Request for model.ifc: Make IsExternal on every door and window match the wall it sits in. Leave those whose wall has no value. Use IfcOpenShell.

First a look at what the model holds.

```python
import ifcopenshell
import ifcopenshell.util.element

model = ifcopenshell.open("model.ifc")
print(model.schema)
seen = {}
for e in model.by_type("IfcDoor") + model.by_type("IfcWindow"):
    if not e.FillsVoids:
        continue
    host = e.FillsVoids[0].RelatingOpeningElement.VoidsElements[0].RelatingBuildingElement
    own = ifcopenshell.util.element.get_pset(e, f"Pset_{e.is_a()[3:].removesuffix('StandardCase')}Common", "IsExternal")
    wall = ifcopenshell.util.element.get_pset(host, "Pset_WallCommon", "IsExternal")
    seen[e.is_a(), own, wall] = seen.get((e.is_a(), own, wall), 0) + 1
for (cls, own, wall), count in sorted(seen.items(), key=str):
    print(count, cls, "IsExternal:", own, "| host wall:", wall)
```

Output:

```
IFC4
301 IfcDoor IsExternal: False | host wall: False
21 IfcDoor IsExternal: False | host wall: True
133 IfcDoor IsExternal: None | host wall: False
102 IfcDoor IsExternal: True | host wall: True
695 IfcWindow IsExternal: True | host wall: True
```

```python
import ifcopenshell
import ifcopenshell.api.pset
import ifcopenshell.util.element

model = ifcopenshell.open("model.ifc")

count = 0
for ifc_class, pset_name in (("IfcDoor", "Pset_DoorCommon"), ("IfcWindow", "Pset_WindowCommon")):
    for e in model.by_type(ifc_class):
        if not e.FillsVoids:
            continue
        host = e.FillsVoids[0].RelatingOpeningElement.VoidsElements[0].RelatingBuildingElement
        external = ifcopenshell.util.element.get_pset(host, "Pset_WallCommon", "IsExternal")
        if external is None or ifcopenshell.util.element.get_pset(e, pset_name, "IsExternal") == external:
            continue
        pset = ifcopenshell.api.pset.add_pset(model, product=e, name=pset_name)
        ifcopenshell.api.pset.edit_pset(model, pset=pset, properties={"IsExternal": external})
        count += 1

print(count, "updated")

model.write("model_edited.ifc")
```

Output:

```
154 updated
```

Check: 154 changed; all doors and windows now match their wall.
